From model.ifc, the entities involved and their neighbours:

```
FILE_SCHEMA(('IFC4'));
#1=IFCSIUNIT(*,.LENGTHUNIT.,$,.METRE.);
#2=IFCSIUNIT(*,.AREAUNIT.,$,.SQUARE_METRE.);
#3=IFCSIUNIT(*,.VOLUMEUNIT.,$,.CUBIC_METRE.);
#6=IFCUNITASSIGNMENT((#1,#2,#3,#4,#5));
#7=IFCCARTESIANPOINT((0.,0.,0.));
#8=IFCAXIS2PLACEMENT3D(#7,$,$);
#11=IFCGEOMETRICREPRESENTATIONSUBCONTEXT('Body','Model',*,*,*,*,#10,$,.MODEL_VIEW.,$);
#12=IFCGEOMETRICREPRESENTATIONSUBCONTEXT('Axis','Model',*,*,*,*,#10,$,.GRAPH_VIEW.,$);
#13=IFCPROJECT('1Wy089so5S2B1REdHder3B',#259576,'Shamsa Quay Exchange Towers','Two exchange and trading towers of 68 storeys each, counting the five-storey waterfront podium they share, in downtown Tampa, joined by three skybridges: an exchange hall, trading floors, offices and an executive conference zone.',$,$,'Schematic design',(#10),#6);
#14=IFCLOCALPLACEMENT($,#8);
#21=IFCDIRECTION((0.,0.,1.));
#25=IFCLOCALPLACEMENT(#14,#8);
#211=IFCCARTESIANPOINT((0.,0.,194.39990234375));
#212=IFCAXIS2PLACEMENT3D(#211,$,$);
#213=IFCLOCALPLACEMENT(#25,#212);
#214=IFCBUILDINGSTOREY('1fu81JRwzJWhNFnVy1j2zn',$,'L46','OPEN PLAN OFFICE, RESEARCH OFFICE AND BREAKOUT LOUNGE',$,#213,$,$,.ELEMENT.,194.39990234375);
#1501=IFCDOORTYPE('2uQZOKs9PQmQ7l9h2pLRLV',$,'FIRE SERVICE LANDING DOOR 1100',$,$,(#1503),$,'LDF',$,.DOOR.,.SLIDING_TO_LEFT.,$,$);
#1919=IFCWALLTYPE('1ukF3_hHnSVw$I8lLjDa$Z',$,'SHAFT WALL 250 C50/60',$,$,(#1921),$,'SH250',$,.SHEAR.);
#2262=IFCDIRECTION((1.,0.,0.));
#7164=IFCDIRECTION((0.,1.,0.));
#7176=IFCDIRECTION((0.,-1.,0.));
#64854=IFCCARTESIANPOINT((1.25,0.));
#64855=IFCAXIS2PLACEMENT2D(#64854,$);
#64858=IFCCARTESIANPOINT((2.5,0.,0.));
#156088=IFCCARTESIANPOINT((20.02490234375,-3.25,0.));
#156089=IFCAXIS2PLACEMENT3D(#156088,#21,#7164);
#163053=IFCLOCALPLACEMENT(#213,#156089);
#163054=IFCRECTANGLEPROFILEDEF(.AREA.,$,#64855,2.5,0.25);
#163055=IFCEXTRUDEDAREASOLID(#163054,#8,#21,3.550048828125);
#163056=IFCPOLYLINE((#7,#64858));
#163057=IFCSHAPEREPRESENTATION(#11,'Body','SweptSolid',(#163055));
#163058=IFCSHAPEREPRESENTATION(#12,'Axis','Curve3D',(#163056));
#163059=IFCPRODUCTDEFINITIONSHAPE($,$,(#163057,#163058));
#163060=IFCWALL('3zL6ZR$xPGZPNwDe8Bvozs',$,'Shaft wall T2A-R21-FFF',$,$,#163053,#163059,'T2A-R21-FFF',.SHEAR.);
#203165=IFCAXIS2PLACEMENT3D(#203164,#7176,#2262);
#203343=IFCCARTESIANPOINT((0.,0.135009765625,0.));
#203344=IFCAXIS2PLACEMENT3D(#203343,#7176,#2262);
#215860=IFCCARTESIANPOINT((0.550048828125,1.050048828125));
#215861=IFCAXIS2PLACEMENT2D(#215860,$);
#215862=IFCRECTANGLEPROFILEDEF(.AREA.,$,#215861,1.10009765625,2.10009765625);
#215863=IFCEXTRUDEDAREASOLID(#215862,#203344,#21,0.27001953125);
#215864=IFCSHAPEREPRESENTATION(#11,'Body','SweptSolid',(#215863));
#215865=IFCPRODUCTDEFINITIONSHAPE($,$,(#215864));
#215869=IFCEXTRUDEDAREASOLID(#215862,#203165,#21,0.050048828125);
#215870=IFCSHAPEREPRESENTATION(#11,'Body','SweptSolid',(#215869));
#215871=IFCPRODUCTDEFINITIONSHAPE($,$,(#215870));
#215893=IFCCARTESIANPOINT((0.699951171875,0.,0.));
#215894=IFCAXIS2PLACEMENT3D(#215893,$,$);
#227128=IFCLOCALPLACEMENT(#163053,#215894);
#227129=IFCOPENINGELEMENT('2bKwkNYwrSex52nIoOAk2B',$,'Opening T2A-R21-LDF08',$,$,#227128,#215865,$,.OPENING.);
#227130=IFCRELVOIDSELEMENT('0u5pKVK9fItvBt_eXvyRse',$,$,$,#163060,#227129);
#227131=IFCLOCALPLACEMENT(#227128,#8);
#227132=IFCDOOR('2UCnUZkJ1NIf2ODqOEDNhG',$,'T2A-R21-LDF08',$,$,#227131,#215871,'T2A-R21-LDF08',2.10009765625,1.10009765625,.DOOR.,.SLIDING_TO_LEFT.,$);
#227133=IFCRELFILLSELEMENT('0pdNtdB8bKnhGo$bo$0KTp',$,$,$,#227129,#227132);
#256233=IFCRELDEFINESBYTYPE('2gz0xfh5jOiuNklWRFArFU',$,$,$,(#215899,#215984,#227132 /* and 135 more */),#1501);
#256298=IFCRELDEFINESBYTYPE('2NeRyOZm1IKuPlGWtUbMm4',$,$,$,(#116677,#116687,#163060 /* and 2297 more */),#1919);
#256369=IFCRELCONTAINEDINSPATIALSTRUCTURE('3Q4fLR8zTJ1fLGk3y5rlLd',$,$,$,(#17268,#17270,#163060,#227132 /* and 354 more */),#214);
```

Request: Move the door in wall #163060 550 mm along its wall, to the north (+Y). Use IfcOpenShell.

```python
import ifcopenshell
import ifcopenshell.api.geometry
import ifcopenshell.util.placement

model = ifcopenshell.open("model.ifc")

door = model.by_id(227132)
opening = door.FillsVoids[0].RelatingOpeningElement
wall = opening.VoidsElements[0].RelatingBuildingElement

wall_matrix = ifcopenshell.util.placement.get_local_placement(wall.ObjectPlacement)
shift = wall_matrix[:3, 0] * 0.55
before = ifcopenshell.util.placement.get_local_placement(door.ObjectPlacement)[:3, 3].copy()

# The door is placed relative to its opening, so it follows when the opening moves.
matrix = ifcopenshell.util.placement.get_local_placement(opening.ObjectPlacement)
matrix[:3, 3] += shift
ifcopenshell.api.geometry.edit_object_placement(
    model, product=opening, matrix=matrix, is_si=False, should_transform_children=True
)

after = ifcopenshell.util.placement.get_local_placement(door.ObjectPlacement)[:3, 3]
print("door moved by", (after - before).round(3) + 0.0)

model.write("model_rev.ifc")
```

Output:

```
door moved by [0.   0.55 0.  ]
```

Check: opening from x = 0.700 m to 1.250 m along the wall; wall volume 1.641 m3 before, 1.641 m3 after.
